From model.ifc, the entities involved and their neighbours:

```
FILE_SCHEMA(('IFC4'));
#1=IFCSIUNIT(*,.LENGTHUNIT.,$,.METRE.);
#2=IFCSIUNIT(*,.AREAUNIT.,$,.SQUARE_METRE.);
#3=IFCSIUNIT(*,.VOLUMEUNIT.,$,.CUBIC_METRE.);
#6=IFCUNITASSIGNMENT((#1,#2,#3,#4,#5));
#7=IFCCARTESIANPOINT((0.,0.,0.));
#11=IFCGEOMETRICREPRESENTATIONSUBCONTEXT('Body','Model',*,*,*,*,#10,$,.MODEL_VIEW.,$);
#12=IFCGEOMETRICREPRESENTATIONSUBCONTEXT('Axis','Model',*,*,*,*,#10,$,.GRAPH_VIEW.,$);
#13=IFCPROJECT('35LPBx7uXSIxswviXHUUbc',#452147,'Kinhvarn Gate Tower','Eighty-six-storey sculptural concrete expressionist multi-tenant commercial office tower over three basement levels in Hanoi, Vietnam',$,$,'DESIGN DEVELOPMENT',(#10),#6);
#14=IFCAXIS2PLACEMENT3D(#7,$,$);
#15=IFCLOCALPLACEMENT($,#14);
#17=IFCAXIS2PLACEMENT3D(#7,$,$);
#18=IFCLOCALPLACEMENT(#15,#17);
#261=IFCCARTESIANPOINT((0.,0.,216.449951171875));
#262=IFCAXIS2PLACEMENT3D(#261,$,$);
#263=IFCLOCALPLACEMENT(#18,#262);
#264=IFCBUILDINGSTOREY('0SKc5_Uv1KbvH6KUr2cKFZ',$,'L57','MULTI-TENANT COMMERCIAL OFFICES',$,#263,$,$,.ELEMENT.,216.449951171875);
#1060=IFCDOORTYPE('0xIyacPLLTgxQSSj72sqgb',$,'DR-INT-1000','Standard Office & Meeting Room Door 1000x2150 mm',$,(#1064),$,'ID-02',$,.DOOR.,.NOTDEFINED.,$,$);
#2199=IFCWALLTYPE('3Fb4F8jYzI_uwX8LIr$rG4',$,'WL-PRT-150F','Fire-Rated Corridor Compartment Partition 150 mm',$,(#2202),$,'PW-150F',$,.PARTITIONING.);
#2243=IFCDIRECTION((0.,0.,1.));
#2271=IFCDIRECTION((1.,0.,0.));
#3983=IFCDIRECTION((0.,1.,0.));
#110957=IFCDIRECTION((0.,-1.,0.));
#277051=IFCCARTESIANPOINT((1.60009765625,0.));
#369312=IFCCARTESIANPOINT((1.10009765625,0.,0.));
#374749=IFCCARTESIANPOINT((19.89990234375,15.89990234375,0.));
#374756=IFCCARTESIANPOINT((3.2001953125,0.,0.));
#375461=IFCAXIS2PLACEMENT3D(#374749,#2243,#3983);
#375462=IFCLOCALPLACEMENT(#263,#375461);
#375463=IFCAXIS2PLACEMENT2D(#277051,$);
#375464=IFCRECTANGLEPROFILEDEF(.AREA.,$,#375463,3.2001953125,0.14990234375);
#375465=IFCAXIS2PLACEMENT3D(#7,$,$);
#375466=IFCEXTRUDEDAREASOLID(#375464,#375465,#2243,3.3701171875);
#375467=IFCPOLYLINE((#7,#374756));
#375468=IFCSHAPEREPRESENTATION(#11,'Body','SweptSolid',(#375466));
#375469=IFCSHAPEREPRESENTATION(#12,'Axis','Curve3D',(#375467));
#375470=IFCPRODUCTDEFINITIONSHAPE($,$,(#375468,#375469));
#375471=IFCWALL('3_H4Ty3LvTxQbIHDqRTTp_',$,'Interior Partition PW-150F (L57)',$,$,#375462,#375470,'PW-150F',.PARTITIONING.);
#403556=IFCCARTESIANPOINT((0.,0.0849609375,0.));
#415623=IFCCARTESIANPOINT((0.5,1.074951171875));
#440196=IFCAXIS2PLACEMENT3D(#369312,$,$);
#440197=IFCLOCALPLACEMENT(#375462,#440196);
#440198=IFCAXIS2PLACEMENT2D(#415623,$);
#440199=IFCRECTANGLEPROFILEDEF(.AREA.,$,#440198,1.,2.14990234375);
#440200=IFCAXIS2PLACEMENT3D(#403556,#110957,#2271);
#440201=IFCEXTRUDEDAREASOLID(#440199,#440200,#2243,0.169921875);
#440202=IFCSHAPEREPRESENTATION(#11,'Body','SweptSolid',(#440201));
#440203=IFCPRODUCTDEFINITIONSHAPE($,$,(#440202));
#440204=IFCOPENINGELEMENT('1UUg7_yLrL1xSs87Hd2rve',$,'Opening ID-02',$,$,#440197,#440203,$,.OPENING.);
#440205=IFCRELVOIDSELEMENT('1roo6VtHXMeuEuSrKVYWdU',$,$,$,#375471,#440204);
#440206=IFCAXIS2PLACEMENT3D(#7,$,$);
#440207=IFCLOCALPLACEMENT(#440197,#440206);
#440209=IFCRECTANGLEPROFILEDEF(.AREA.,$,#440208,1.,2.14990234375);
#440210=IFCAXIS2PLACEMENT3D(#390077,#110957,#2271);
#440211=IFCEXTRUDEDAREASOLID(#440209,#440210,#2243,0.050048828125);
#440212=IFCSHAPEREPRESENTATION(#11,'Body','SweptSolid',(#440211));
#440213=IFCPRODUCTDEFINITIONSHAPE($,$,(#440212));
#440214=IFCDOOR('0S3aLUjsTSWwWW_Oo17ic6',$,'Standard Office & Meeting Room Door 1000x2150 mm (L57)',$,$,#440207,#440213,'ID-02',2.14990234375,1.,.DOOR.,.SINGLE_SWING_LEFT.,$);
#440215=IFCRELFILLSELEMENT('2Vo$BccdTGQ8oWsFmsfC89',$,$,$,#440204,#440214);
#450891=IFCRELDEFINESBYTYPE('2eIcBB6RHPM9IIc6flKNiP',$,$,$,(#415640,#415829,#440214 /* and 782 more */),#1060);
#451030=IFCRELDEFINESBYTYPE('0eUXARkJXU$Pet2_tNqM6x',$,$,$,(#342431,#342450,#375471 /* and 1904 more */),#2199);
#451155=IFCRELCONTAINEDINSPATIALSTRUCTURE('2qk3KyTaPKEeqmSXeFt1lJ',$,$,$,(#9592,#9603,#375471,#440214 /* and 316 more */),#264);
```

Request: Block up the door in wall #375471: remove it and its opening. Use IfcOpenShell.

```python
import ifcopenshell
import ifcopenshell.api.feature
import ifcopenshell.api.root
import ifcopenshell.geom
import ifcopenshell.util.shape

model = ifcopenshell.open("model.ifc")
settings = ifcopenshell.geom.settings()


def volume(element):
    """Net volume in cubic metres, openings subtracted."""
    shape = ifcopenshell.geom.create_shape(settings, element)
    return ifcopenshell.util.shape.get_volume(shape.geometry)


door = model.by_guid("0S3aLUjsTSWwWW_Oo17ic6")
opening = door.FillsVoids[0].RelatingOpeningElement
wall = opening.VoidsElements[0].RelatingBuildingElement
before = volume(wall)

ifcopenshell.api.root.remove_product(model, product=door)
ifcopenshell.api.feature.remove_feature(model, feature=opening)

after = volume(wall)

print(f"wall volume {before:.3f} -> {after:.3f} m3")

model.write("model-out.ifc")
```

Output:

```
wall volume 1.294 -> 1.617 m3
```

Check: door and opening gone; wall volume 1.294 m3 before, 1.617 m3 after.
